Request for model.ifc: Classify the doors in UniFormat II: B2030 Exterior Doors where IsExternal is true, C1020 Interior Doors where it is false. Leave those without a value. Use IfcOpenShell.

First a look at what the model holds.

```python
import ifcopenshell
import ifcopenshell.util.element

model = ifcopenshell.open("model.ifc")
print(model.schema)
print("classifications:", [c.Name for c in model.by_type("IfcClassification")])
values = [ifcopenshell.util.element.get_pset(e, "Pset_DoorCommon", "IsExternal") for e in model.by_type("IfcDoor")]
for value in (True, False, None):
    print("IsExternal", value, values.count(value))
```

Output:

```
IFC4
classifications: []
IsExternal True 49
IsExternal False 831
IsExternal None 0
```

```python
import ifcopenshell
import ifcopenshell.api.classification
import ifcopenshell.util.element

model = ifcopenshell.open("model.ifc")

system = ifcopenshell.api.classification.add_classification(model, classification="UniFormat II")

doors = model.by_type("IfcDoor")
external = {e: ifcopenshell.util.element.get_pset(e, "Pset_DoorCommon", "IsExternal") for e in doors}
for flag, code, name in ((True, "B2030", "Exterior Doors"), (False, "C1020", "Interior Doors")):
    products = [e for e in doors if external[e] is flag]
    ifcopenshell.api.classification.add_reference(
        model, products=products, classification=system, identification=code, name=name
    )
    print(code, len(products))

model.write("model_edited.ifc")
```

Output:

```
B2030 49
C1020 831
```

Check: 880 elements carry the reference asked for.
